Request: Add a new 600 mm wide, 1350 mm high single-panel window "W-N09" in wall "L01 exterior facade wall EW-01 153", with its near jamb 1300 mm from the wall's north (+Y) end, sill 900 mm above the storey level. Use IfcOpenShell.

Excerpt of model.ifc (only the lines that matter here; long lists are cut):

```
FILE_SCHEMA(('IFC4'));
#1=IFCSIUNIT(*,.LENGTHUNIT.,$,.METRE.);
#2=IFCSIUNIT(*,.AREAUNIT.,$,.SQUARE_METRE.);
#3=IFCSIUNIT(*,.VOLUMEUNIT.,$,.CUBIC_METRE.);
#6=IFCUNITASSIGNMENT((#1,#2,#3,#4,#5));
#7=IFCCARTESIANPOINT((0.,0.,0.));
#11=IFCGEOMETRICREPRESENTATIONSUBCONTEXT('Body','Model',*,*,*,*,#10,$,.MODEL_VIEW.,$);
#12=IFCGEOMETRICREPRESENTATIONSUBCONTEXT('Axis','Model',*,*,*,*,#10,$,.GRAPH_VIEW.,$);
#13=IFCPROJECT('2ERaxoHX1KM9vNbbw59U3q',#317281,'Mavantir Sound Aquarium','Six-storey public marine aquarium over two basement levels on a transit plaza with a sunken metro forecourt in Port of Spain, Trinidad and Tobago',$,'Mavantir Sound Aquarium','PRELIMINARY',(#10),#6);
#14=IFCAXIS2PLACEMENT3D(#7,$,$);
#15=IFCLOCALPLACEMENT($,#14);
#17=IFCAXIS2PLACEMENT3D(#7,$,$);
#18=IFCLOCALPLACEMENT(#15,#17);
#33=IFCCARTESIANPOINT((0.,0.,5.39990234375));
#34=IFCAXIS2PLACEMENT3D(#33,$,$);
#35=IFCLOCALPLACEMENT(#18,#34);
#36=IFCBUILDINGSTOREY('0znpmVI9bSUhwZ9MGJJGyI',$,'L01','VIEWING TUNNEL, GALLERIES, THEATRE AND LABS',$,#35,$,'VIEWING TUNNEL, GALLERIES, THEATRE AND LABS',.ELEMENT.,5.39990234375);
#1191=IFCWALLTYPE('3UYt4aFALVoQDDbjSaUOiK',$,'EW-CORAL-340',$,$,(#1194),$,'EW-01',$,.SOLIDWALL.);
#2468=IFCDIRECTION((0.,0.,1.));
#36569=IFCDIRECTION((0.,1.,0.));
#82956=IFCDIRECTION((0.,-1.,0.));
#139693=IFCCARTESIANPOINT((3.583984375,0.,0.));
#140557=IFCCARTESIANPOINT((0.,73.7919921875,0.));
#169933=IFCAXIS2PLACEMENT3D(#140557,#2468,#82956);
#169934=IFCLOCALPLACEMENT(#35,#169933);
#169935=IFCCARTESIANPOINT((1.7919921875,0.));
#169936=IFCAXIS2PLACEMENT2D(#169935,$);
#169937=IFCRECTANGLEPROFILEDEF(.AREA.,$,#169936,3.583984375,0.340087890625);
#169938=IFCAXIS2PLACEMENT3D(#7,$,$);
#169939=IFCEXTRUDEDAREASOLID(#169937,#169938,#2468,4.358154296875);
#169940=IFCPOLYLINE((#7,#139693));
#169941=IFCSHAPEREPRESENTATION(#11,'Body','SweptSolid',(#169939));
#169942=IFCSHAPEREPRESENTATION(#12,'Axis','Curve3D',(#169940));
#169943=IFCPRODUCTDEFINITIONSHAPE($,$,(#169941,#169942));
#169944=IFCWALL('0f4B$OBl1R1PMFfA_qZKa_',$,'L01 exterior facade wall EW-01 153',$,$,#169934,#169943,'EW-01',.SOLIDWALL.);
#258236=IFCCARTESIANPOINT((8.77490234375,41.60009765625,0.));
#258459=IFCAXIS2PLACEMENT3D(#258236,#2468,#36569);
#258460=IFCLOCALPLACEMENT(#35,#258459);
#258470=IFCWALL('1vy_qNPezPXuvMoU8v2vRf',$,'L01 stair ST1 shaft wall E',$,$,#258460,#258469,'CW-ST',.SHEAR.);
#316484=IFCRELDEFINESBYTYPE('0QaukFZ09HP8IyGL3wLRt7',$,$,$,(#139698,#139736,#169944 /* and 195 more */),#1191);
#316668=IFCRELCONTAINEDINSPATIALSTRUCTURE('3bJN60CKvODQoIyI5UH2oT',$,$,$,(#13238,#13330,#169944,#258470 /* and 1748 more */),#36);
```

```python
import numpy as np
import ifcopenshell
import ifcopenshell.api.feature
import ifcopenshell.api.geometry
import ifcopenshell.api.root
import ifcopenshell.api.spatial
import ifcopenshell.geom
import ifcopenshell.util.element
import ifcopenshell.util.placement
import ifcopenshell.util.representation
import ifcopenshell.util.shape
import ifcopenshell.util.unit

model = ifcopenshell.open("model.ifc")
unit_scale = ifcopenshell.util.unit.calculate_unit_scale(model)
settings = ifcopenshell.geom.settings()


def volume(element):
    """Net volume in cubic metres, openings subtracted."""
    shape = ifcopenshell.geom.create_shape(settings, element)
    return ifcopenshell.util.shape.get_volume(shape.geometry)


wall = model.by_guid("0f4B$OBl1R1PMFfA_qZKa_")
storey = ifcopenshell.util.element.get_container(wall, ifc_class="IfcBuildingStorey")
context = ifcopenshell.util.representation.get_context(model, "Model", "Body", "MODEL_VIEW")
before = volume(wall)

width, height, from_end, sill = 0.6, 1.35, 1.3, 0.9  # metres

# The wall runs along its own X axis, and the end named is its -X end.
wall_shape = ifcopenshell.geom.create_shape(settings, wall)
x, y, z = ifcopenshell.util.shape.get_vertices(wall_shape.geometry).T
start = x.min() + from_end
face, thickness = float(y.min()), float(y.max() - y.min())
wall_matrix = ifcopenshell.util.placement.get_local_placement(wall.ObjectPlacement)
level = ifcopenshell.util.placement.get_local_placement(storey.ObjectPlacement)[2, 3]


def in_wall(x, y):
    """Placement at x, y metres in the wall's axes, at sill height."""
    matrix = wall_matrix.copy()
    matrix[:, 3] = wall_matrix @ np.array([x / unit_scale, y / unit_scale, 0.0, 1.0])
    matrix[2, 3] = level + sill / unit_scale
    return matrix


# Opening: a box that overshoots both wall faces by 50 mm.
opening = ifcopenshell.api.root.create_entity(model, ifc_class="IfcOpeningElement", predefined_type="OPENING")
box = ifcopenshell.api.geometry.add_wall_representation(
    model, context=context, length=width, height=height, thickness=thickness + 0.1
)
ifcopenshell.api.geometry.assign_representation(model, product=opening, representation=box)
ifcopenshell.api.geometry.edit_object_placement(model, product=opening, matrix=in_wall(start, face - 0.05), is_si=False)
ifcopenshell.api.feature.add_feature(model, feature=opening, element=wall)

window = ifcopenshell.api.root.create_entity(model, ifc_class="IfcWindow", name="W-N09", predefined_type="WINDOW")
window.OverallWidth, window.OverallHeight = width / unit_scale, height / unit_scale
window.PartitioningType = "SINGLE_PANEL"
body = ifcopenshell.api.geometry.add_window_representation(
    model,
    context=context,
    overall_width=window.OverallWidth,
    overall_height=window.OverallHeight,
    partition_type="SINGLE_PANEL",
)
ifcopenshell.api.geometry.assign_representation(model, product=window, representation=body)
ifcopenshell.api.spatial.assign_container(model, products=[window], relating_structure=storey)
ifcopenshell.api.feature.add_filling(model, opening=opening, element=window)

# Centre the window in the wall's thickness.
ifcopenshell.api.geometry.edit_object_placement(model, product=window, matrix=in_wall(start, face), is_si=False)
window_shape = ifcopenshell.geom.create_shape(settings, window)
depth = ifcopenshell.util.shape.get_vertices(window_shape.geometry)[:, 1]
offset = face + thickness / 2 - (depth.min() + depth.max()) / 2
ifcopenshell.api.geometry.edit_object_placement(model, product=window, matrix=in_wall(start, offset), is_si=False)

after = volume(wall)

print(f"wall volume {before:.3f} -> {after:.3f} m3")

model.write("model-out.ifc")
```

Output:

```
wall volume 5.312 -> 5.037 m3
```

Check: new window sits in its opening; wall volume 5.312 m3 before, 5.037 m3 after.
